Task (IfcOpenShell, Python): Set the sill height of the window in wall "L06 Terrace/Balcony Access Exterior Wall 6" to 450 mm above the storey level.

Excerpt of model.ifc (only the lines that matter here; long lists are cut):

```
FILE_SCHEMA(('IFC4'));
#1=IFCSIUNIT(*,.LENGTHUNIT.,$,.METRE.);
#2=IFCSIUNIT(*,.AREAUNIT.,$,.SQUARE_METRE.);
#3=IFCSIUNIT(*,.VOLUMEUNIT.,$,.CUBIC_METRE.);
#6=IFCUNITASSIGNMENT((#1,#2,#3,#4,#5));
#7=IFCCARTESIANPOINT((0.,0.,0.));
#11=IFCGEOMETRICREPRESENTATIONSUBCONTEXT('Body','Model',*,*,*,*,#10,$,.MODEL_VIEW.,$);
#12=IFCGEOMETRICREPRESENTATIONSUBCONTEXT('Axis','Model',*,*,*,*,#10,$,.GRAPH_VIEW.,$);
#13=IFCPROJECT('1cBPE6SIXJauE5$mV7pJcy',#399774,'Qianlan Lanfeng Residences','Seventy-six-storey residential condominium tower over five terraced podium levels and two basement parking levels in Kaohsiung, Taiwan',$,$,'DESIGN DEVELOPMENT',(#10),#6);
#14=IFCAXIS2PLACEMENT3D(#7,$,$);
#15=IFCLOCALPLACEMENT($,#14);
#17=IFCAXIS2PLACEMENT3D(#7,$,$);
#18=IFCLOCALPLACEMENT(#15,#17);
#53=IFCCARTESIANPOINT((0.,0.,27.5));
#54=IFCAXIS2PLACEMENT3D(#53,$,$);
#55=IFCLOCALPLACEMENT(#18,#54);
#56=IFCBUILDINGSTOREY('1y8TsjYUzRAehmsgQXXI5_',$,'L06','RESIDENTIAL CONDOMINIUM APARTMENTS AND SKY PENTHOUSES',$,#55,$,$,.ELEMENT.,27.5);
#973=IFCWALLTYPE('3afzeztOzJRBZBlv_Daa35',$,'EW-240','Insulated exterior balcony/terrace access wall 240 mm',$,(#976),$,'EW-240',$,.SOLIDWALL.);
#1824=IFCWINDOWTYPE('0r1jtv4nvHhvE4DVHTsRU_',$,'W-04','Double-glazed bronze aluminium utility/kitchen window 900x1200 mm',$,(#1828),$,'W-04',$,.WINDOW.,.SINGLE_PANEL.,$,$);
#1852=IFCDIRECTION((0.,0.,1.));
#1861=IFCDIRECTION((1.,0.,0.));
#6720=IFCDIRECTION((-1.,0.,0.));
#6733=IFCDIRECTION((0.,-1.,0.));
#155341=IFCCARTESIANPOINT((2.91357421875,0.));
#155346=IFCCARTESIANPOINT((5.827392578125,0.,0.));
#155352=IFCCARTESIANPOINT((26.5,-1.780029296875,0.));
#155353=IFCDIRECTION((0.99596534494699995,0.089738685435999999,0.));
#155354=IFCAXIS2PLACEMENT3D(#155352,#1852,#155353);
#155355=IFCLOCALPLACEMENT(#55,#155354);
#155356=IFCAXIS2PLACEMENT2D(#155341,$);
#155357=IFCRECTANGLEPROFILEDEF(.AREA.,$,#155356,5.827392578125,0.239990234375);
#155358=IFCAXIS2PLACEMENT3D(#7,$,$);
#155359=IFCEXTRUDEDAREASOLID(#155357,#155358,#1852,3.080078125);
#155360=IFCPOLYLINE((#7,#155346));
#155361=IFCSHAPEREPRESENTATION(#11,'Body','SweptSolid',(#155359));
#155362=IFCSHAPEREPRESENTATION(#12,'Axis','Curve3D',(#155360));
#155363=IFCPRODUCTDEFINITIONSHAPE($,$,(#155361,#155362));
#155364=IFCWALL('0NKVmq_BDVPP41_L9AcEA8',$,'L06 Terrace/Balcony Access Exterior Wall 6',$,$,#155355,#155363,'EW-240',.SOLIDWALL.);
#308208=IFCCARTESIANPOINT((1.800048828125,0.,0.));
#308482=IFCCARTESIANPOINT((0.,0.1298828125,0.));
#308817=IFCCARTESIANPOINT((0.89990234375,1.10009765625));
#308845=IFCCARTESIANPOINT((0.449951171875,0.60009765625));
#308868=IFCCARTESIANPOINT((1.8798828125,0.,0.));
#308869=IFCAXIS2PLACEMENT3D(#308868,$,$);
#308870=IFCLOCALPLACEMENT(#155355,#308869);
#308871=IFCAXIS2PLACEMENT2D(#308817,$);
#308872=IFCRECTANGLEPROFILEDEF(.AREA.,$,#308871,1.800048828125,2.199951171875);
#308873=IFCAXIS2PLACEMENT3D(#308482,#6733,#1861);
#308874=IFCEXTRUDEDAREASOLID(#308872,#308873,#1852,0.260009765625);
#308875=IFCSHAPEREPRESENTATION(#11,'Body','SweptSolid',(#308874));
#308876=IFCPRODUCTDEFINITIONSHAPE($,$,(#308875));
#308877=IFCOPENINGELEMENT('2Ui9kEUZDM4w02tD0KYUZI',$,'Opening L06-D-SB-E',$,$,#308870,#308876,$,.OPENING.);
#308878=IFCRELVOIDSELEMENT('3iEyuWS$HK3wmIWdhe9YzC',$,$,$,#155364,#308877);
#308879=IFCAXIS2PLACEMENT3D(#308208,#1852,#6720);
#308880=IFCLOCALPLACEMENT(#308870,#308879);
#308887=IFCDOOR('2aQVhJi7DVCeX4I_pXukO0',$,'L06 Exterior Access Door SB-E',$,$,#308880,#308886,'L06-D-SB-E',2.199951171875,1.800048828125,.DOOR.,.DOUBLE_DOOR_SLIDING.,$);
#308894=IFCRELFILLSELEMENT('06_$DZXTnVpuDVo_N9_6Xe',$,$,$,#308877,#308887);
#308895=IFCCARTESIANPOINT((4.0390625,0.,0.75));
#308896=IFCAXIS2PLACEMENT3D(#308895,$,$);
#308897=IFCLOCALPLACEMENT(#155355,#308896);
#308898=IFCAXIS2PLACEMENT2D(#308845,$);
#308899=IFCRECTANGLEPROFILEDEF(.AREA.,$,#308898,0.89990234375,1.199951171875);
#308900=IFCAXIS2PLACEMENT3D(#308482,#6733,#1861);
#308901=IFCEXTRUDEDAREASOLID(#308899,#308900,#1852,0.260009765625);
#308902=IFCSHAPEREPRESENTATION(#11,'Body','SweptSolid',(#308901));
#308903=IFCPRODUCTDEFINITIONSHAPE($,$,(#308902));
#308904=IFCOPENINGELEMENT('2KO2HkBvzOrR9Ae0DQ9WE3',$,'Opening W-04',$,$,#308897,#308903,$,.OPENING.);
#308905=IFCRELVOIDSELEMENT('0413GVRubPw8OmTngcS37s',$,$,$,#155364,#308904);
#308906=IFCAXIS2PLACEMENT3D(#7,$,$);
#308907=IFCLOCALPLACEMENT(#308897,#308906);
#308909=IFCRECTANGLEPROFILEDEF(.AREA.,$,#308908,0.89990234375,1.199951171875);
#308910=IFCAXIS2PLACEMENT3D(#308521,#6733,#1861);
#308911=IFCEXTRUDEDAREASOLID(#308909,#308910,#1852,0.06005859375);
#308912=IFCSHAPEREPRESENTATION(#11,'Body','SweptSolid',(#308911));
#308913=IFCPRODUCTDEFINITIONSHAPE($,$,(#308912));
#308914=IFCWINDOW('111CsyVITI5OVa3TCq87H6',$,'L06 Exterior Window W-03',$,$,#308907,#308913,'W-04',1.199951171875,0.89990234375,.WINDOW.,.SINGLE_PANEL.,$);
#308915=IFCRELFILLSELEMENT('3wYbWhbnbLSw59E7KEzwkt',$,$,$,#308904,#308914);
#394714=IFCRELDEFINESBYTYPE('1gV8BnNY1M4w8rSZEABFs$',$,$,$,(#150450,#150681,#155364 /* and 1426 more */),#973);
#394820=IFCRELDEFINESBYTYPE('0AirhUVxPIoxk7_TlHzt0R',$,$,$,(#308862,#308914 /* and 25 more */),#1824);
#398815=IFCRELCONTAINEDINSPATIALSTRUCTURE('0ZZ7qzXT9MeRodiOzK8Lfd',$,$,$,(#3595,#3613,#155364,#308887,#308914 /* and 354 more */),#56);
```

```python
import numpy as np
import ifcopenshell
import ifcopenshell.api.geometry
import ifcopenshell.geom
import ifcopenshell.util.element
import ifcopenshell.util.placement
import ifcopenshell.util.shape
import ifcopenshell.util.unit

model = ifcopenshell.open("model.ifc")
unit_scale = ifcopenshell.util.unit.calculate_unit_scale(model)

window = model.by_guid("111CsyVITI5OVa3TCq87H6")
opening = window.FillsVoids[0].RelatingOpeningElement
storey = ifcopenshell.util.element.get_container(window, ifc_class="IfcBuildingStorey")
level = ifcopenshell.util.placement.get_local_placement(storey.ObjectPlacement)[2, 3]

# The opening's origin need not be at the sill, so measure its lowest point.
shape = ifcopenshell.geom.create_shape(ifcopenshell.geom.settings(), opening)
bottom = ifcopenshell.util.shape.get_shape_bottom_elevation(shape, shape.geometry) / unit_scale
dz = level + 0.45 / unit_scale - bottom

shift = np.array([0.0, 0.0, dz])
# The window is placed relative to its opening, so it follows when the opening moves.
matrix = ifcopenshell.util.placement.get_local_placement(opening.ObjectPlacement)
matrix[:3, 3] += shift
ifcopenshell.api.geometry.edit_object_placement(
    model, product=opening, matrix=matrix, is_si=False, should_transform_children=True
)

print(f"moved by {dz * unit_scale:+.3f} m")

model.write("model_edited.ifc")
```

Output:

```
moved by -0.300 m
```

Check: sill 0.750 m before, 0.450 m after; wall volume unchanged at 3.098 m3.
